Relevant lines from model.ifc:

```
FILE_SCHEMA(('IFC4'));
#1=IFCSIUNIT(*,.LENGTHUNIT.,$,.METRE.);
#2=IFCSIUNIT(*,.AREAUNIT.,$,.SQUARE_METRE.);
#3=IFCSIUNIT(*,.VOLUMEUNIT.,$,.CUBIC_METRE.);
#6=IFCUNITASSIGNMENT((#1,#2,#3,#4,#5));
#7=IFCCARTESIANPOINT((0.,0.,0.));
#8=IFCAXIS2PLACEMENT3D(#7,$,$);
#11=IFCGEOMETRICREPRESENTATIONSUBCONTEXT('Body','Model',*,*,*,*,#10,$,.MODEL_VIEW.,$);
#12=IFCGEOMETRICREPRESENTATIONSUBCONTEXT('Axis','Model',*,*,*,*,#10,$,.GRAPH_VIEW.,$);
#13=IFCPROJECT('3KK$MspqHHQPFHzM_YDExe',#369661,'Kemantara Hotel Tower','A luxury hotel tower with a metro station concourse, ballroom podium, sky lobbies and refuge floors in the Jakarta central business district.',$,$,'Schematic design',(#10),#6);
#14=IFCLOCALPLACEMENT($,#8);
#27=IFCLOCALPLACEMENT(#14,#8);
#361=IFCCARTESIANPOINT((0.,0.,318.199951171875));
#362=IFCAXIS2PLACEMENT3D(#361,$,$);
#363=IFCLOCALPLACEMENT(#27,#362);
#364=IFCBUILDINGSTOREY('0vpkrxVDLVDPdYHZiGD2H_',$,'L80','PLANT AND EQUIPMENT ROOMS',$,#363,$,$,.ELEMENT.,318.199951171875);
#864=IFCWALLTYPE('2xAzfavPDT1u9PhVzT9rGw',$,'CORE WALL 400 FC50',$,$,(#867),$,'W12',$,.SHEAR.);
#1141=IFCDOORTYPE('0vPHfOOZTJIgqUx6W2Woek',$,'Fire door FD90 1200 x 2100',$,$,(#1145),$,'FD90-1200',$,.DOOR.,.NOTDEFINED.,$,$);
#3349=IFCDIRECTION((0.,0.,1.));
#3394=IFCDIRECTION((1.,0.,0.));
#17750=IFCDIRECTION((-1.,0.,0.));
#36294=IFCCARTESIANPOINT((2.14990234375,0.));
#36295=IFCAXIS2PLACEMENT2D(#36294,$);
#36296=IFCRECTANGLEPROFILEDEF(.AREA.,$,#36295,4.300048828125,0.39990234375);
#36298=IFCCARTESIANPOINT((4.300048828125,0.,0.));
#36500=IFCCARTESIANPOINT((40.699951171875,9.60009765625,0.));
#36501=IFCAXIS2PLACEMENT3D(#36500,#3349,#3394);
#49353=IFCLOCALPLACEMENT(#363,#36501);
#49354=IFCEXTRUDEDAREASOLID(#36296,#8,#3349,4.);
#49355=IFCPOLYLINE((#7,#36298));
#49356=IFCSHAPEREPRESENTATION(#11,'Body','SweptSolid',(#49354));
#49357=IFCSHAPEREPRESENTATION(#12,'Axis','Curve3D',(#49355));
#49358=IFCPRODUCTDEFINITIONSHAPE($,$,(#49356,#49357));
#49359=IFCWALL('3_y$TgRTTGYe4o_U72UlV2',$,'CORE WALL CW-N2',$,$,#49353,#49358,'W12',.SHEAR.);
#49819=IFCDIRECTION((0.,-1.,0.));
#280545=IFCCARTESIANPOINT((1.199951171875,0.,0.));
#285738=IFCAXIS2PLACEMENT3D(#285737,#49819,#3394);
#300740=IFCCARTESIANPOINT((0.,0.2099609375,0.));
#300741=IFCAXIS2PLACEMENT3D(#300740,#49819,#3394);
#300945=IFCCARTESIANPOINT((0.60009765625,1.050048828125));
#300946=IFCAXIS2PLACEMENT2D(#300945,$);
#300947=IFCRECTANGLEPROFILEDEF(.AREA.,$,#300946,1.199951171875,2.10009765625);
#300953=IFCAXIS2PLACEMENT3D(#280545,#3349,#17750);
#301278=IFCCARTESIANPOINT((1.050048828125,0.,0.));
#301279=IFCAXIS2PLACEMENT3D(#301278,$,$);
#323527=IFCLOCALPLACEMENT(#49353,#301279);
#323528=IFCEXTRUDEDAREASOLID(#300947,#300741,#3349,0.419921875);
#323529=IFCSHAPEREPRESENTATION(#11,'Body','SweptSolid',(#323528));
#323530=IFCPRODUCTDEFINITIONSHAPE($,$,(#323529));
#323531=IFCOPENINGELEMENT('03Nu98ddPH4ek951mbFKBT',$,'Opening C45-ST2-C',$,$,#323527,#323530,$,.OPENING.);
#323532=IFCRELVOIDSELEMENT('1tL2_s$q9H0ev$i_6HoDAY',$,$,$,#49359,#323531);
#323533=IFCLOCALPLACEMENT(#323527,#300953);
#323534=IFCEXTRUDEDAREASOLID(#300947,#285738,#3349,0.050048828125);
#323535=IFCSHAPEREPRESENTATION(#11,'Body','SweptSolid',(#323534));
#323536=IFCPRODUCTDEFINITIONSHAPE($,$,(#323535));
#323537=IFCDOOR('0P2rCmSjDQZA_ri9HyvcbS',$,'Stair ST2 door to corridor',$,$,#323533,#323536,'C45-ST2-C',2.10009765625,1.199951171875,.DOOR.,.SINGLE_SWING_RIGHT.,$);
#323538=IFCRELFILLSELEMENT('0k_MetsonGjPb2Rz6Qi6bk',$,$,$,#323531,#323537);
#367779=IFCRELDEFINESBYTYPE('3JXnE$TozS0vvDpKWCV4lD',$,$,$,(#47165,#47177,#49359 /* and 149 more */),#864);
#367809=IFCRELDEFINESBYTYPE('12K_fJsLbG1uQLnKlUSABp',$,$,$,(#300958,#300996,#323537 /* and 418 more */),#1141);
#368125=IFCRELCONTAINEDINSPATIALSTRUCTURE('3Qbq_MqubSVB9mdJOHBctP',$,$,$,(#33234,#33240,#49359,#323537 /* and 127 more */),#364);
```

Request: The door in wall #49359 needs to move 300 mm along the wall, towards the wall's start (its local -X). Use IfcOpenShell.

```python
import ifcopenshell
import ifcopenshell.api.geometry
import ifcopenshell.util.placement

model = ifcopenshell.open("model.ifc")

door = model.by_id(323537)
opening = door.FillsVoids[0].RelatingOpeningElement
wall = opening.VoidsElements[0].RelatingBuildingElement

wall_matrix = ifcopenshell.util.placement.get_local_placement(wall.ObjectPlacement)
shift = wall_matrix[:3, 0] * -0.3
before = ifcopenshell.util.placement.get_local_placement(door.ObjectPlacement)[:3, 3].copy()

# The door is placed relative to its opening, so it follows when the opening moves.
matrix = ifcopenshell.util.placement.get_local_placement(opening.ObjectPlacement)
matrix[:3, 3] += shift
ifcopenshell.api.geometry.edit_object_placement(
    model, product=opening, matrix=matrix, is_si=False, should_transform_children=True
)

after = ifcopenshell.util.placement.get_local_placement(door.ObjectPlacement)[:3, 3]
print("door moved by", (after - before).round(3) + 0.0)

model.write("model-out.ifc")
```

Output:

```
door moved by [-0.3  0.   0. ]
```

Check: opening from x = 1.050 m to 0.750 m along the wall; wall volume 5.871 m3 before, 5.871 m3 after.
